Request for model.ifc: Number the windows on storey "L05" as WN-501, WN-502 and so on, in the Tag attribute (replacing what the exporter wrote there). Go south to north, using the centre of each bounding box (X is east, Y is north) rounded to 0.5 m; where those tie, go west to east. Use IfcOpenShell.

First a look at what the model holds.

```python
import ifcopenshell
import ifcopenshell.util.element
import ifcopenshell.util.placement

model = ifcopenshell.open("model.ifc")
print(model.schema)
storey = next(s for s in model.by_type("IfcBuildingStorey") if s.Name == "L05")
windows = [e for e in ifcopenshell.util.element.get_decomposition(storey) if e.is_a("IfcWindow")]
for e in sorted(windows, key=lambda e: e.id()):
    origin = ifcopenshell.util.placement.get_local_placement(e.ObjectPlacement)[:3, 3]
    print(e.id(), e.Tag, e.Name, origin.round(2) + 0.0, sep=" | ")
```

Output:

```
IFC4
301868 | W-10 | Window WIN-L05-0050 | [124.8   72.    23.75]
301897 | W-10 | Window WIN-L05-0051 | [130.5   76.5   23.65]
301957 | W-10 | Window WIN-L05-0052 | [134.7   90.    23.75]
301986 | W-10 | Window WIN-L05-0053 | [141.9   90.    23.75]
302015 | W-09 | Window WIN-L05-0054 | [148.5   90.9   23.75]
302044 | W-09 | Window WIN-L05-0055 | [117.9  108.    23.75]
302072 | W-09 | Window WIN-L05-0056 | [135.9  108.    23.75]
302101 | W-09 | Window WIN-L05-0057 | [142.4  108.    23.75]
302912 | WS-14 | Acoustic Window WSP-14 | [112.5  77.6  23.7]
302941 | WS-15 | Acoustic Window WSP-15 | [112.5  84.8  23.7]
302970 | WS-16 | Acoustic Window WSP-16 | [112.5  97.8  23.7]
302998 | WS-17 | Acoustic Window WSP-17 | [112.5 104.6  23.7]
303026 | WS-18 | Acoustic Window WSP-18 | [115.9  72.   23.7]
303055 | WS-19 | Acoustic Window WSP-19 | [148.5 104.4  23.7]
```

```python
import ifcopenshell
import ifcopenshell.geom
import ifcopenshell.util.element
import ifcopenshell.util.shape

model = ifcopenshell.open("model.ifc")
settings = ifcopenshell.geom.settings()
settings.set("use-world-coords", True)


def centre(element):
    shape = ifcopenshell.geom.create_shape(settings, element)
    return ifcopenshell.util.shape.get_bbox_centroid(shape.geometry)


storey = next(s for s in model.by_type("IfcBuildingStorey") if s.Name == "L05")
windows = [e for e in ifcopenshell.util.element.get_decomposition(storey) if e.is_a("IfcWindow")]

# Insertion points can sit at a corner or the storey origin, so sort by the geometry (in metres).
centres = {e: centre(e) for e in windows}
windows.sort(key=lambda e: (round(centres[e][1] / 0.5), centres[e][0]))

for i, e in enumerate(windows, start=1):
    number = f"WN-5{i:02d}"
    e.Tag = number
    print(e.id(), number)

model.write("model-out.ifc")
```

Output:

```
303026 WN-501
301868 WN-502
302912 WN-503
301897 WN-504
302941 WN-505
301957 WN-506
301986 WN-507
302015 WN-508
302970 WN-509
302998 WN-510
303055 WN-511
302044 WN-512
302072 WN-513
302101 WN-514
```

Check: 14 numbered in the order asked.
